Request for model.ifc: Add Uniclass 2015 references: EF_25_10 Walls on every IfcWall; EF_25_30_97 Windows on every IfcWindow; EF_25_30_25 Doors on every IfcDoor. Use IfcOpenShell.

First a look at what the model holds.

```python
import ifcopenshell

model = ifcopenshell.open("model.ifc")
print(model.schema)
print("classifications:", [c.Name for c in model.by_type("IfcClassification")])
for ifc_class in ("IfcDoor", "IfcRoof", "IfcStair", "IfcWall", "IfcWindow"):
    print(ifc_class, len(model.by_type(ifc_class)))
```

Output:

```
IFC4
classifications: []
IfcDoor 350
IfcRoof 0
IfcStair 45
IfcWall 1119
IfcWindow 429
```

```python
import ifcopenshell
import ifcopenshell.api.classification

model = ifcopenshell.open("model.ifc")

system = ifcopenshell.api.classification.add_classification(model, classification="Uniclass 2015")

codes = {
    "IfcWall": ("EF_25_10", "Walls"),
    "IfcWindow": ("EF_25_30_97", "Windows"),
    "IfcDoor": ("EF_25_30_25", "Doors"),
}
for ifc_class, (code, name) in codes.items():
    products = model.by_type(ifc_class)
    ifcopenshell.api.classification.add_reference(
        model, products=products, classification=system, identification=code, name=name
    )
    print(code, len(products))

model.write("model_v2.ifc")
```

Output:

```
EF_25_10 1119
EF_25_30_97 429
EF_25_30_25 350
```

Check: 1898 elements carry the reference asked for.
